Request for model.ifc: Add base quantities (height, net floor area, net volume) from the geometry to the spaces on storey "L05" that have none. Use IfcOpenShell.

First a look at what the model holds.

```python
import ifcopenshell
import ifcopenshell.util.element
import ifcopenshell.util.unit

model = ifcopenshell.open("model.ifc")
print(model.schema)
for unit_type in ("LENGTHUNIT", "AREAUNIT", "VOLUMEUNIT"):
    print(unit_type, ifcopenshell.util.unit.calculate_unit_scale(model, unit_type))
storey = next(s for s in model.by_type("IfcBuildingStorey") if s.Name == "L05")
spaces = [e for e in ifcopenshell.util.element.get_decomposition(storey) if e.is_a("IfcSpace")]
for e in sorted(spaces, key=lambda e: e.id()):
    print(e.id(), e.is_a(), e.Name, list(ifcopenshell.util.element.get_psets(e, qtos_only=True)), sep=" | ")
```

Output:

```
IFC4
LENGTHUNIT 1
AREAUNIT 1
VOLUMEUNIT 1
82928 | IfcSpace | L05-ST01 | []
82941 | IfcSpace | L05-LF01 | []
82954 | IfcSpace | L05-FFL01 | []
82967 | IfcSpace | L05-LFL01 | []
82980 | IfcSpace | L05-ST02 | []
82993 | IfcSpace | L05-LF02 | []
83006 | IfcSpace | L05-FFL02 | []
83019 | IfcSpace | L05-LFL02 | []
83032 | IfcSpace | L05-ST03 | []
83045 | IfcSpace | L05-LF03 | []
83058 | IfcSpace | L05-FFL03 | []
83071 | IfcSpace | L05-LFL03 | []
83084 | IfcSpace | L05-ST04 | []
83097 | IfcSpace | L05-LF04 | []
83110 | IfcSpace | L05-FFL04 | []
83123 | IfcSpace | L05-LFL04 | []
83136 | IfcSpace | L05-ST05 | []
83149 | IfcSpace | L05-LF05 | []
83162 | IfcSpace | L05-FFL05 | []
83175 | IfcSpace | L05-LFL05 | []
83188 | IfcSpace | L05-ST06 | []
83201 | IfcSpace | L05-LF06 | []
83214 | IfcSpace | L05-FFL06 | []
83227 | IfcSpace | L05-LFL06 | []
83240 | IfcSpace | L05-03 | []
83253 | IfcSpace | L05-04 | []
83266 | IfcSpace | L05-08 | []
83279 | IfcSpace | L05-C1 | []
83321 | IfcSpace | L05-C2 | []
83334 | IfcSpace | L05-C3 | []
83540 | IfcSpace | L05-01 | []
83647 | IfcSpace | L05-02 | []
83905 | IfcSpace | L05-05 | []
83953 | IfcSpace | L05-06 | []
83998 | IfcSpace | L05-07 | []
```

```python
import ifcopenshell
import ifcopenshell.api.pset
import ifcopenshell.geom
import ifcopenshell.util.element
import ifcopenshell.util.shape
import ifcopenshell.util.unit

model = ifcopenshell.open("model.ifc")
unit_scale = ifcopenshell.util.unit.calculate_unit_scale(model)
area_scale = ifcopenshell.util.unit.calculate_unit_scale(model, "AREAUNIT")
volume_scale = ifcopenshell.util.unit.calculate_unit_scale(model, "VOLUMEUNIT")
settings = ifcopenshell.geom.settings()

storey = next(s for s in model.by_type("IfcBuildingStorey") if s.Name == "L05")
spaces = [e for e in ifcopenshell.util.element.get_decomposition(storey) if e.is_a("IfcSpace")]

for e in sorted(spaces, key=lambda e: e.id()):
    if ifcopenshell.util.element.get_psets(e, qtos_only=True, should_inherit=False):
        continue
    # Geometry comes back in metres, in the element's own axes.
    shape = ifcopenshell.geom.create_shape(settings, e)
    values = {
        "Height": ifcopenshell.util.shape.get_z(shape.geometry) / unit_scale,
        "NetFloorArea": ifcopenshell.util.shape.get_footprint_area(shape.geometry) / area_scale,
        "NetVolume": ifcopenshell.util.shape.get_volume(shape.geometry) / volume_scale,
    }
    qto = ifcopenshell.api.pset.add_qto(model, product=e, name="Qto_SpaceBaseQuantities")
    ifcopenshell.api.pset.edit_qto(model, qto=qto, properties=values)
    print(e.id(), {k: round(v, 3) for k, v in values.items()})

model.write("model-out.ifc")
```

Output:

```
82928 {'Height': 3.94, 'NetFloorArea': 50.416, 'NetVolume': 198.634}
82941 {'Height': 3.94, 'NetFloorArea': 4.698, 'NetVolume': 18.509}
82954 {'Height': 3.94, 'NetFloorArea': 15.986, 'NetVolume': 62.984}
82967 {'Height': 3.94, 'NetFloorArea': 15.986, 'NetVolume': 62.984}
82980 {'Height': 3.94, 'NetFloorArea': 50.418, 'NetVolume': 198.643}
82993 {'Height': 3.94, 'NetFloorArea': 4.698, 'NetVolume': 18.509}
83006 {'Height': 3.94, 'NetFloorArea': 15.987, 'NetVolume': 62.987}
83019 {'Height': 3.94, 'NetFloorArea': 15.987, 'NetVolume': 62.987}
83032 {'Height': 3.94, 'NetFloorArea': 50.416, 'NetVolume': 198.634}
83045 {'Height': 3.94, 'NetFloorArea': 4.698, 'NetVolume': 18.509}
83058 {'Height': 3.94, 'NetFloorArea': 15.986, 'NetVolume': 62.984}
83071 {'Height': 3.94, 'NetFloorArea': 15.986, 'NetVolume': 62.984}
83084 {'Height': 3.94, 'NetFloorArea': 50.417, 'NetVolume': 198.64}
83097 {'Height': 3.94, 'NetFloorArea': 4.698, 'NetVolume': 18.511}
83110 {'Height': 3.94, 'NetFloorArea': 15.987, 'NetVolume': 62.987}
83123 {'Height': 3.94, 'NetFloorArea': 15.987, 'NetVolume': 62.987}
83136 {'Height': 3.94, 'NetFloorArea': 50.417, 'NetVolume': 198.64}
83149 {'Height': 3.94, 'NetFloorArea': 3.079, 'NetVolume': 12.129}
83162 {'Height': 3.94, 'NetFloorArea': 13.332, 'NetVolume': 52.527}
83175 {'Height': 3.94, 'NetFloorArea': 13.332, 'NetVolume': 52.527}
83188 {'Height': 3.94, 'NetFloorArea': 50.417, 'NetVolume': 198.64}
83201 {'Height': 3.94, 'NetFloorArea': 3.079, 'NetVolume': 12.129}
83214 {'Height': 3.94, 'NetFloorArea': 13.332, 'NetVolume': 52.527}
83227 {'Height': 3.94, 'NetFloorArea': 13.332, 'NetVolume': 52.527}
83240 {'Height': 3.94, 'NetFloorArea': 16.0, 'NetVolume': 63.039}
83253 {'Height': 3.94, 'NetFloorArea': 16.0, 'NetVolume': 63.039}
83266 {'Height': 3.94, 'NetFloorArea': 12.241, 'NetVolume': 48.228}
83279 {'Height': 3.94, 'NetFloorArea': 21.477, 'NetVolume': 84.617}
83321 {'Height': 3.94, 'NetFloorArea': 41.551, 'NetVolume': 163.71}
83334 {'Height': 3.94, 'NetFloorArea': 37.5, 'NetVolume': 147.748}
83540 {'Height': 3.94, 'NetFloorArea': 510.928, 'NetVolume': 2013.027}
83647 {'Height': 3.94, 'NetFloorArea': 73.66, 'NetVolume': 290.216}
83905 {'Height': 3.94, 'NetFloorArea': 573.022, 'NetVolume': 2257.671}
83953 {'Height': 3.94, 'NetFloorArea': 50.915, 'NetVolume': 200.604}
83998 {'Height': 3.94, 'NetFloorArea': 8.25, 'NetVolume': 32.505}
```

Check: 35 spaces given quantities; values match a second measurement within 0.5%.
